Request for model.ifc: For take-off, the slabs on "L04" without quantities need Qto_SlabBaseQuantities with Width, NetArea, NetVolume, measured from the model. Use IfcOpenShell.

First a look at what the model holds.

```python
import ifcopenshell
import ifcopenshell.util.element
import ifcopenshell.util.unit

model = ifcopenshell.open("model.ifc")
print(model.schema)
for unit_type in ("LENGTHUNIT", "AREAUNIT", "VOLUMEUNIT"):
    print(unit_type, ifcopenshell.util.unit.calculate_unit_scale(model, unit_type))
storey = next(s for s in model.by_type("IfcBuildingStorey") if s.Name == "L04")
slabs = [e for e in ifcopenshell.util.element.get_decomposition(storey) if e.is_a("IfcSlab")]
for e in sorted(slabs, key=lambda e: e.id()):
    print(e.id(), e.is_a(), e.Name, list(ifcopenshell.util.element.get_psets(e, qtos_only=True)), sep=" | ")
```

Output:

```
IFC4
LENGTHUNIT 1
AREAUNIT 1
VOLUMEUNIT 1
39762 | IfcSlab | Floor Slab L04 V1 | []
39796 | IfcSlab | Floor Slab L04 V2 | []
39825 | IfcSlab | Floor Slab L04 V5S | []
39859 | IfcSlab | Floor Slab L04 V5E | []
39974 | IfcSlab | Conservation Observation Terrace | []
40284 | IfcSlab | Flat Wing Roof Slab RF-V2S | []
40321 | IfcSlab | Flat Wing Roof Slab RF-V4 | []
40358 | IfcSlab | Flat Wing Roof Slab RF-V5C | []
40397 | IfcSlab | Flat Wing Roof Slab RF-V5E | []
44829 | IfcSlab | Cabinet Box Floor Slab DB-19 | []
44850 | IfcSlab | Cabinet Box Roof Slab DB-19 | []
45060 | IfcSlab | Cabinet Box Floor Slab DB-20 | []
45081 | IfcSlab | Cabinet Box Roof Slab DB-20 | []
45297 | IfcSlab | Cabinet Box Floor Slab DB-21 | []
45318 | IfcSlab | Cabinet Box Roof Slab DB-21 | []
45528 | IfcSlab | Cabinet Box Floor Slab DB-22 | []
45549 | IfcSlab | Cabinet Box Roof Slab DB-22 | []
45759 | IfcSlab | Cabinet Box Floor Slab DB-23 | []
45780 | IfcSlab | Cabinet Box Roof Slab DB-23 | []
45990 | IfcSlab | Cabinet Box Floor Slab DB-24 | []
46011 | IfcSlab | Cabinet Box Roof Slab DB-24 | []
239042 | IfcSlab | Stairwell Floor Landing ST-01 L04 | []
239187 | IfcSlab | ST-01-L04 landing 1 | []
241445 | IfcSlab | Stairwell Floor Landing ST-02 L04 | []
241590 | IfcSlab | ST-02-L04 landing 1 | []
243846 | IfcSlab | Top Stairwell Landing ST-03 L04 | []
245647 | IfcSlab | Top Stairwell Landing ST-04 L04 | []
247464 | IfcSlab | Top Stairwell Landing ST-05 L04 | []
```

```python
import ifcopenshell
import ifcopenshell.api.pset
import ifcopenshell.geom
import ifcopenshell.util.element
import ifcopenshell.util.shape
import ifcopenshell.util.unit

model = ifcopenshell.open("model.ifc")
unit_scale = ifcopenshell.util.unit.calculate_unit_scale(model)
area_scale = ifcopenshell.util.unit.calculate_unit_scale(model, "AREAUNIT")
volume_scale = ifcopenshell.util.unit.calculate_unit_scale(model, "VOLUMEUNIT")
settings = ifcopenshell.geom.settings()

storey = next(s for s in model.by_type("IfcBuildingStorey") if s.Name == "L04")
slabs = [e for e in ifcopenshell.util.element.get_decomposition(storey) if e.is_a("IfcSlab")]

for e in sorted(slabs, key=lambda e: e.id()):
    if ifcopenshell.util.element.get_psets(e, qtos_only=True, should_inherit=False):
        continue
    # Geometry comes back in metres, in the element's own axes.
    shape = ifcopenshell.geom.create_shape(settings, e)
    values = {
        "Width": ifcopenshell.util.shape.get_z(shape.geometry) / unit_scale,
        "NetArea": ifcopenshell.util.shape.get_footprint_area(shape.geometry) / area_scale,
        "NetVolume": ifcopenshell.util.shape.get_volume(shape.geometry) / volume_scale,
    }
    qto = ifcopenshell.api.pset.add_qto(model, product=e, name="Qto_SlabBaseQuantities")
    ifcopenshell.api.pset.edit_qto(model, qto=qto, properties=values)
    print(e.id(), {k: round(v, 3) for k, v in values.items()})

model.write("model_v2.ifc")
```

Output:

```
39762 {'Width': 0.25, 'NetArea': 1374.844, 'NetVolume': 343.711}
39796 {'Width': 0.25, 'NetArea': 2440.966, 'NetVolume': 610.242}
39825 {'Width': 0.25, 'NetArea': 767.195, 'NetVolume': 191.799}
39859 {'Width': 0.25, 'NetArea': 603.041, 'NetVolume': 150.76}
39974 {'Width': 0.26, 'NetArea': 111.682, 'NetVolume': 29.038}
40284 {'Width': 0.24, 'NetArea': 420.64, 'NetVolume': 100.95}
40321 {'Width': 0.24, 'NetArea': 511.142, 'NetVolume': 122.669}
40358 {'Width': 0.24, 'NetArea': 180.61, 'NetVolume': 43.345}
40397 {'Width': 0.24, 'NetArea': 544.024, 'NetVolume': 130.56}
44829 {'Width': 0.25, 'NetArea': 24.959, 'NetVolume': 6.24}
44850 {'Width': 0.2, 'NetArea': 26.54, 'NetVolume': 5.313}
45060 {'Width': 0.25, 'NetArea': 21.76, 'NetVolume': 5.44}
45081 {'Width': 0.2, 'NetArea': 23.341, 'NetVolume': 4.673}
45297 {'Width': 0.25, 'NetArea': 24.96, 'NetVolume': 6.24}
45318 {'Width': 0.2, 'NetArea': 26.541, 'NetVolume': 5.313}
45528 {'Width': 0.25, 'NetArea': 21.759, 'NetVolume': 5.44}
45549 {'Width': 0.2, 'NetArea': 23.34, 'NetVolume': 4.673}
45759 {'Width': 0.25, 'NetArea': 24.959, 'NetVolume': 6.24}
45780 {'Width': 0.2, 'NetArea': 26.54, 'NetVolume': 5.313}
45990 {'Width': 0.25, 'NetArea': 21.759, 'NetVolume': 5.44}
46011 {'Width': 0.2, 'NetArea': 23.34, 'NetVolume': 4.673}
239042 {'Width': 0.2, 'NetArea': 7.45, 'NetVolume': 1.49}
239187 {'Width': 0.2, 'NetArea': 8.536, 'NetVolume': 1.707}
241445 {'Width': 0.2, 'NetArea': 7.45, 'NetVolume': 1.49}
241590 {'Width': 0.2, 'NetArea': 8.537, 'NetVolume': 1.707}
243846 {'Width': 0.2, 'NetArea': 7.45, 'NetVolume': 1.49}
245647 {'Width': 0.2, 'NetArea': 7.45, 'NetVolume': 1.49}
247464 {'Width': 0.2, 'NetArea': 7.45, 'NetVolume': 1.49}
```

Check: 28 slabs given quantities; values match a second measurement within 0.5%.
